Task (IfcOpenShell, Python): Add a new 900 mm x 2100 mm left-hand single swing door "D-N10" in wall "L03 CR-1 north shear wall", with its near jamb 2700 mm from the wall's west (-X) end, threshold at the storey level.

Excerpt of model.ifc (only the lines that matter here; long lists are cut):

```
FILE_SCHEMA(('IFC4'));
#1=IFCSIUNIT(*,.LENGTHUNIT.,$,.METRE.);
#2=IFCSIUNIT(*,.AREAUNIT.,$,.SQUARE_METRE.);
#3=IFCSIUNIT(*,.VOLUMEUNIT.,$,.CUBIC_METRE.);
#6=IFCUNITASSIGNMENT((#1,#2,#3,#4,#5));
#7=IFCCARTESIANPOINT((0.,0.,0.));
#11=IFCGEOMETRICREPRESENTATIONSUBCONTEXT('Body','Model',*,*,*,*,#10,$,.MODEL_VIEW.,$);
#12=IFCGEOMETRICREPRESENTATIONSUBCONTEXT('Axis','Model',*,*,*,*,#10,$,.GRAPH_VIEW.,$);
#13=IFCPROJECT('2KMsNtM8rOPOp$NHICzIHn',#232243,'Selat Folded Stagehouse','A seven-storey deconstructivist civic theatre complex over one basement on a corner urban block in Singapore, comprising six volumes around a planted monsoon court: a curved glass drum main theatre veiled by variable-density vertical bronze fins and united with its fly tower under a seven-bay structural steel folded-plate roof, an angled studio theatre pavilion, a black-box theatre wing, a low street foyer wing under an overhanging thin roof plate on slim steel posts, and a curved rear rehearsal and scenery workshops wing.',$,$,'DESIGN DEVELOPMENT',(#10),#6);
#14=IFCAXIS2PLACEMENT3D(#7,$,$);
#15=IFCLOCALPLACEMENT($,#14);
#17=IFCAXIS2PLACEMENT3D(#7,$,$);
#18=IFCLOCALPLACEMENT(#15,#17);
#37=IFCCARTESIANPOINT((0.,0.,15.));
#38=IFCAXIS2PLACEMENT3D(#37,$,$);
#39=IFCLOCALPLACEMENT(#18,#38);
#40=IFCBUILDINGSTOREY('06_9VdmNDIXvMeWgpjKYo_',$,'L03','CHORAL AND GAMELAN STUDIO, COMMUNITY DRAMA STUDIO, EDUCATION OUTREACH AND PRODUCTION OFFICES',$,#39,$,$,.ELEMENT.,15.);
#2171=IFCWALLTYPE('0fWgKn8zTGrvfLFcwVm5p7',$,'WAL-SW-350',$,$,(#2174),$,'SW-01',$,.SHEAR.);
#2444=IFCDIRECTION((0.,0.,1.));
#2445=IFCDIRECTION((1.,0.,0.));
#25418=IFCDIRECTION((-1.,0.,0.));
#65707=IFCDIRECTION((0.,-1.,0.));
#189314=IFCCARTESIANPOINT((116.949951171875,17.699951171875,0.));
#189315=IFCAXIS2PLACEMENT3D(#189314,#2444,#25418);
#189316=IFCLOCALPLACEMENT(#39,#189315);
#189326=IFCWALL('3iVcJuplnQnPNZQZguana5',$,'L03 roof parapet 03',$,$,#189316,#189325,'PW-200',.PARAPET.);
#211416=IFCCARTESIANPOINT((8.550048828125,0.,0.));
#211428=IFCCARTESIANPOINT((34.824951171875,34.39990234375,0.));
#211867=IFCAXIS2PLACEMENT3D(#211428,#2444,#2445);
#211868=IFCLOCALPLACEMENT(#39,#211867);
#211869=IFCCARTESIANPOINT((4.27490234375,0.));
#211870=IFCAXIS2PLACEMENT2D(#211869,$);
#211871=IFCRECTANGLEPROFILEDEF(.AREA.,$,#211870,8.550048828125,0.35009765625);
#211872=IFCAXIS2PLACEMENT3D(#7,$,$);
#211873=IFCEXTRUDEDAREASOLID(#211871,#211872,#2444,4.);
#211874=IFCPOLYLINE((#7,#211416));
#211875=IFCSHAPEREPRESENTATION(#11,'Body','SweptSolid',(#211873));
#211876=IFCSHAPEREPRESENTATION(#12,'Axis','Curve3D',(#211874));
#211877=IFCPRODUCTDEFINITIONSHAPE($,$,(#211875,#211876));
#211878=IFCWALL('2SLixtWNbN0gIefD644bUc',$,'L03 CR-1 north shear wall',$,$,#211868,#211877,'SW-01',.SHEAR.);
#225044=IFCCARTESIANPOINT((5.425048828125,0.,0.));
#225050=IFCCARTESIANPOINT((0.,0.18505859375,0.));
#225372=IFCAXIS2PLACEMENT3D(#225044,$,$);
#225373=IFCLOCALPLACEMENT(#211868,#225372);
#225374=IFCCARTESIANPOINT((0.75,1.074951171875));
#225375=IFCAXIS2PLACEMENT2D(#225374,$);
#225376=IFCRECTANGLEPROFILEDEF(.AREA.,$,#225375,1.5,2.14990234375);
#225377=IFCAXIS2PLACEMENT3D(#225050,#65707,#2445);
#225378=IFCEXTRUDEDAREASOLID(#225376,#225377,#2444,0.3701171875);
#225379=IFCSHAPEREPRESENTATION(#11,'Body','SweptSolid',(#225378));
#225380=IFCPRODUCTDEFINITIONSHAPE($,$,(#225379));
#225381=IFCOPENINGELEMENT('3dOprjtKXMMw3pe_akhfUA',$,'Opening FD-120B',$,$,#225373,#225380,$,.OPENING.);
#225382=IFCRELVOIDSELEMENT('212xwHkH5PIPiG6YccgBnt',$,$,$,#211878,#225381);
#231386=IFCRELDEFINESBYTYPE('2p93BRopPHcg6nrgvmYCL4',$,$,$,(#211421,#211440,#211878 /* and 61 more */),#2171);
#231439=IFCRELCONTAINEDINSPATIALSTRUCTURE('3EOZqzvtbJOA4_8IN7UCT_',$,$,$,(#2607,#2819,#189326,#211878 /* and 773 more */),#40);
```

```python
import numpy as np
import ifcopenshell
import ifcopenshell.api.feature
import ifcopenshell.api.geometry
import ifcopenshell.api.root
import ifcopenshell.api.spatial
import ifcopenshell.geom
import ifcopenshell.util.element
import ifcopenshell.util.placement
import ifcopenshell.util.representation
import ifcopenshell.util.shape
import ifcopenshell.util.unit

model = ifcopenshell.open("model.ifc")
unit_scale = ifcopenshell.util.unit.calculate_unit_scale(model)
settings = ifcopenshell.geom.settings()


def volume(element):
    """Net volume in cubic metres, openings subtracted."""
    shape = ifcopenshell.geom.create_shape(settings, element)
    return ifcopenshell.util.shape.get_volume(shape.geometry)


wall = model.by_guid("2SLixtWNbN0gIefD644bUc")
storey = ifcopenshell.util.element.get_container(wall, ifc_class="IfcBuildingStorey")
context = ifcopenshell.util.representation.get_context(model, "Model", "Body", "MODEL_VIEW")
before = volume(wall)

width, height, from_end, sill = 0.9, 2.1, 2.7, 0.0  # metres

# The wall runs along its own X axis, and the end named is its -X end.
wall_shape = ifcopenshell.geom.create_shape(settings, wall)
x, y, z = ifcopenshell.util.shape.get_vertices(wall_shape.geometry).T
start = x.min() + from_end
face, thickness = float(y.min()), float(y.max() - y.min())
wall_matrix = ifcopenshell.util.placement.get_local_placement(wall.ObjectPlacement)
level = ifcopenshell.util.placement.get_local_placement(storey.ObjectPlacement)[2, 3]


def in_wall(x, y):
    """Placement at x, y metres in the wall's axes, at sill height."""
    matrix = wall_matrix.copy()
    matrix[:, 3] = wall_matrix @ np.array([x / unit_scale, y / unit_scale, 0.0, 1.0])
    matrix[2, 3] = level + sill / unit_scale
    return matrix


# Opening: a box that overshoots both wall faces by 50 mm.
opening = ifcopenshell.api.root.create_entity(model, ifc_class="IfcOpeningElement", predefined_type="OPENING")
box = ifcopenshell.api.geometry.add_wall_representation(
    model, context=context, length=width, height=height, thickness=thickness + 0.1
)
ifcopenshell.api.geometry.assign_representation(model, product=opening, representation=box)
ifcopenshell.api.geometry.edit_object_placement(model, product=opening, matrix=in_wall(start, face - 0.05), is_si=False)
ifcopenshell.api.feature.add_feature(model, feature=opening, element=wall)

door = ifcopenshell.api.root.create_entity(model, ifc_class="IfcDoor", name="D-N10", predefined_type="DOOR")
door.OverallWidth, door.OverallHeight = width / unit_scale, height / unit_scale
door.OperationType = "SINGLE_SWING_LEFT"
body = ifcopenshell.api.geometry.add_door_representation(
    model,
    context=context,
    overall_width=door.OverallWidth,
    overall_height=door.OverallHeight,
    operation_type="SINGLE_SWING_LEFT",
    lining_properties={"LiningDepth": thickness / unit_scale, "ThresholdDepth": thickness / unit_scale},
)
ifcopenshell.api.geometry.assign_representation(model, product=door, representation=body)
ifcopenshell.api.spatial.assign_container(model, products=[door], relating_structure=storey)
ifcopenshell.api.feature.add_filling(model, opening=opening, element=door)

# The lining spans the wall, so the door starts at the wall face.
ifcopenshell.api.geometry.edit_object_placement(model, product=door, matrix=in_wall(start, face), is_si=False)

after = volume(wall)

print(f"wall volume {before:.3f} -> {after:.3f} m3")

model.write("model_v2.ifc")
```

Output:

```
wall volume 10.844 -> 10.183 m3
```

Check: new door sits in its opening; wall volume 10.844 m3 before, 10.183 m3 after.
